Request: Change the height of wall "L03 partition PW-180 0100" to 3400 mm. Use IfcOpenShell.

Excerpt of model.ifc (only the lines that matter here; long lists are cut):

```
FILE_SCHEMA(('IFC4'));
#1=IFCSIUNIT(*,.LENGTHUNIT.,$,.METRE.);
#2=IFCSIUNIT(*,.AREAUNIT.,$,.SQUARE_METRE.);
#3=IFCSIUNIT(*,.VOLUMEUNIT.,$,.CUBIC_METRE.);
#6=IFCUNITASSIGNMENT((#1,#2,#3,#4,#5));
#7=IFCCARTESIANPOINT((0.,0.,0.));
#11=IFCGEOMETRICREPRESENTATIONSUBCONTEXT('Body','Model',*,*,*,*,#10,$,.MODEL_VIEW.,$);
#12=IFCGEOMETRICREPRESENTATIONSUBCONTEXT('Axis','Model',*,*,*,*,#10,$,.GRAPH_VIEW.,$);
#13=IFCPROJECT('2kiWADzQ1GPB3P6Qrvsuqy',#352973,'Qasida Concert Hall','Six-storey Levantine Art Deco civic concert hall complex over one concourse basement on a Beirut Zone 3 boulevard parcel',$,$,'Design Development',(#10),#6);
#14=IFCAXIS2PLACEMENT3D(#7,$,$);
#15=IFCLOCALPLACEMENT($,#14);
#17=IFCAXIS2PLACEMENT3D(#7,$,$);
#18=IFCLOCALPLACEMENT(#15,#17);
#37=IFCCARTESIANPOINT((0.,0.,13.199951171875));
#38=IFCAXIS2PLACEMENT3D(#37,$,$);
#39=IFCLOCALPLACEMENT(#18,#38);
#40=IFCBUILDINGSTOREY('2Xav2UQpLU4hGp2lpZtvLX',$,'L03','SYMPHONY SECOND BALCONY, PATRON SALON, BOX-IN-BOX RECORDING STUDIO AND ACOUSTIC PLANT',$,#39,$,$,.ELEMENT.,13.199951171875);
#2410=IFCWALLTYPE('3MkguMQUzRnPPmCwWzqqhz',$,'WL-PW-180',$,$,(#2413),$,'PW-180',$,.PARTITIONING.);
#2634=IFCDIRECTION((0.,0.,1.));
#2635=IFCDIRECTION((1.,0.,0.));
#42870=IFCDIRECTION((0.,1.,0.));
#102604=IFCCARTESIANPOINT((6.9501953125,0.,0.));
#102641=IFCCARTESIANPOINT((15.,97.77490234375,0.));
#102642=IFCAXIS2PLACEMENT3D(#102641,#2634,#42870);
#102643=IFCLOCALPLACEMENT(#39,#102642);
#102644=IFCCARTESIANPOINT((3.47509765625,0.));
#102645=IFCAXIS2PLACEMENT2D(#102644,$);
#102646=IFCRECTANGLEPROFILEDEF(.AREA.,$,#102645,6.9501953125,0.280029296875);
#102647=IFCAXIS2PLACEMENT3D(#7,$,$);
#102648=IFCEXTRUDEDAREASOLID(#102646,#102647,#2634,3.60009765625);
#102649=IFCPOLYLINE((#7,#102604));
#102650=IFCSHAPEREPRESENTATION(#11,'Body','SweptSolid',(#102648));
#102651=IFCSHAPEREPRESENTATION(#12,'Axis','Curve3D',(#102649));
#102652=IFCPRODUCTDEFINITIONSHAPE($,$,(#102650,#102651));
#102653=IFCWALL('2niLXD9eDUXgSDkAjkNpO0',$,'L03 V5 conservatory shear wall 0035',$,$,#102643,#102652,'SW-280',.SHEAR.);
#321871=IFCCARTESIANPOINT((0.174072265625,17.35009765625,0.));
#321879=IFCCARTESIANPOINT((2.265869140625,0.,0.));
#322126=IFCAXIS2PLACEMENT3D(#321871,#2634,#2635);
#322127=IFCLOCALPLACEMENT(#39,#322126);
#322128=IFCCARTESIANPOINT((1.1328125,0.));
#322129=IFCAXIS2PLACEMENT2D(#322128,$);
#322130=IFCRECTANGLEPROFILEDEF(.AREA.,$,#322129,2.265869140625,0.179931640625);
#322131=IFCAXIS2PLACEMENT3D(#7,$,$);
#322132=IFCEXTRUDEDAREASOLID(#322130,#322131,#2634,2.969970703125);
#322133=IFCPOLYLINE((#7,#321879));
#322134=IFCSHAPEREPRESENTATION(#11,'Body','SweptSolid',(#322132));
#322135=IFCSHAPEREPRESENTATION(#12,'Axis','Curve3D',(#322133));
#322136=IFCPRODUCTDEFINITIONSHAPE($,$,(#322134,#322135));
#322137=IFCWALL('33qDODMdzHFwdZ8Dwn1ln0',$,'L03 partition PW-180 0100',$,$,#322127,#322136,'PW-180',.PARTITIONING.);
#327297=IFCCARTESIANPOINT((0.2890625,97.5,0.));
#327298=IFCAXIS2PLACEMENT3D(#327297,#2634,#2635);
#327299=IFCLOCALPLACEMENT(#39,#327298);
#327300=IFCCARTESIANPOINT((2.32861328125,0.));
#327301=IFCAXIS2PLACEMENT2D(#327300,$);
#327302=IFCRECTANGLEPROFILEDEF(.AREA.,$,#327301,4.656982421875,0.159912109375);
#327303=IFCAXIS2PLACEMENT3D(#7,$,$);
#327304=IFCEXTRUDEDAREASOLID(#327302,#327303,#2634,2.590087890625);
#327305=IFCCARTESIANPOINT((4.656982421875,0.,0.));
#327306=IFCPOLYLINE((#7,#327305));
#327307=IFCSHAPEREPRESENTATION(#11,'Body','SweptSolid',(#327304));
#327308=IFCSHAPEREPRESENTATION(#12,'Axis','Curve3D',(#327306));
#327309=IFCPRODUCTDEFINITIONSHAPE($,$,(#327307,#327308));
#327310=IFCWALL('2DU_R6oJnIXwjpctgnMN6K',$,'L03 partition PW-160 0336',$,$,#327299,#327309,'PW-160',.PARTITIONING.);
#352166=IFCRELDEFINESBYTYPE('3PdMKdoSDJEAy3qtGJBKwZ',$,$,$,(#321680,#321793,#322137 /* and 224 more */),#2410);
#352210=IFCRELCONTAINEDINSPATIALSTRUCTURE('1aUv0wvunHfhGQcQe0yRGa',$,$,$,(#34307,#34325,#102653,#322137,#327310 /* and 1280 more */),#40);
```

```python
import ifcopenshell
import ifcopenshell.geom
import ifcopenshell.util.representation
import ifcopenshell.util.shape
import ifcopenshell.util.unit

model = ifcopenshell.open("model.ifc")
unit_scale = ifcopenshell.util.unit.calculate_unit_scale(model)
settings = ifcopenshell.geom.settings()


def volume(element):
    """Net volume in cubic metres, openings subtracted."""
    shape = ifcopenshell.geom.create_shape(settings, element)
    return ifcopenshell.util.shape.get_volume(shape.geometry)


wall = model.by_guid("33qDODMdzHFwdZ8Dwn1ln0")
before = volume(wall)

body = ifcopenshell.util.representation.get_representation(wall, "Model", "Body")
solid = body.Items[0]
old_height = solid.Depth
solid.Depth = 3.4 / unit_scale
after = volume(wall)

print(f"height {old_height:g} -> {solid.Depth:g}, volume {before:.3f} -> {after:.3f} m3")

model.write("model_rev.ifc")
```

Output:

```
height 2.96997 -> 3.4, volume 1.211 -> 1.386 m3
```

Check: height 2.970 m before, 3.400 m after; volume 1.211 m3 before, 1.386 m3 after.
